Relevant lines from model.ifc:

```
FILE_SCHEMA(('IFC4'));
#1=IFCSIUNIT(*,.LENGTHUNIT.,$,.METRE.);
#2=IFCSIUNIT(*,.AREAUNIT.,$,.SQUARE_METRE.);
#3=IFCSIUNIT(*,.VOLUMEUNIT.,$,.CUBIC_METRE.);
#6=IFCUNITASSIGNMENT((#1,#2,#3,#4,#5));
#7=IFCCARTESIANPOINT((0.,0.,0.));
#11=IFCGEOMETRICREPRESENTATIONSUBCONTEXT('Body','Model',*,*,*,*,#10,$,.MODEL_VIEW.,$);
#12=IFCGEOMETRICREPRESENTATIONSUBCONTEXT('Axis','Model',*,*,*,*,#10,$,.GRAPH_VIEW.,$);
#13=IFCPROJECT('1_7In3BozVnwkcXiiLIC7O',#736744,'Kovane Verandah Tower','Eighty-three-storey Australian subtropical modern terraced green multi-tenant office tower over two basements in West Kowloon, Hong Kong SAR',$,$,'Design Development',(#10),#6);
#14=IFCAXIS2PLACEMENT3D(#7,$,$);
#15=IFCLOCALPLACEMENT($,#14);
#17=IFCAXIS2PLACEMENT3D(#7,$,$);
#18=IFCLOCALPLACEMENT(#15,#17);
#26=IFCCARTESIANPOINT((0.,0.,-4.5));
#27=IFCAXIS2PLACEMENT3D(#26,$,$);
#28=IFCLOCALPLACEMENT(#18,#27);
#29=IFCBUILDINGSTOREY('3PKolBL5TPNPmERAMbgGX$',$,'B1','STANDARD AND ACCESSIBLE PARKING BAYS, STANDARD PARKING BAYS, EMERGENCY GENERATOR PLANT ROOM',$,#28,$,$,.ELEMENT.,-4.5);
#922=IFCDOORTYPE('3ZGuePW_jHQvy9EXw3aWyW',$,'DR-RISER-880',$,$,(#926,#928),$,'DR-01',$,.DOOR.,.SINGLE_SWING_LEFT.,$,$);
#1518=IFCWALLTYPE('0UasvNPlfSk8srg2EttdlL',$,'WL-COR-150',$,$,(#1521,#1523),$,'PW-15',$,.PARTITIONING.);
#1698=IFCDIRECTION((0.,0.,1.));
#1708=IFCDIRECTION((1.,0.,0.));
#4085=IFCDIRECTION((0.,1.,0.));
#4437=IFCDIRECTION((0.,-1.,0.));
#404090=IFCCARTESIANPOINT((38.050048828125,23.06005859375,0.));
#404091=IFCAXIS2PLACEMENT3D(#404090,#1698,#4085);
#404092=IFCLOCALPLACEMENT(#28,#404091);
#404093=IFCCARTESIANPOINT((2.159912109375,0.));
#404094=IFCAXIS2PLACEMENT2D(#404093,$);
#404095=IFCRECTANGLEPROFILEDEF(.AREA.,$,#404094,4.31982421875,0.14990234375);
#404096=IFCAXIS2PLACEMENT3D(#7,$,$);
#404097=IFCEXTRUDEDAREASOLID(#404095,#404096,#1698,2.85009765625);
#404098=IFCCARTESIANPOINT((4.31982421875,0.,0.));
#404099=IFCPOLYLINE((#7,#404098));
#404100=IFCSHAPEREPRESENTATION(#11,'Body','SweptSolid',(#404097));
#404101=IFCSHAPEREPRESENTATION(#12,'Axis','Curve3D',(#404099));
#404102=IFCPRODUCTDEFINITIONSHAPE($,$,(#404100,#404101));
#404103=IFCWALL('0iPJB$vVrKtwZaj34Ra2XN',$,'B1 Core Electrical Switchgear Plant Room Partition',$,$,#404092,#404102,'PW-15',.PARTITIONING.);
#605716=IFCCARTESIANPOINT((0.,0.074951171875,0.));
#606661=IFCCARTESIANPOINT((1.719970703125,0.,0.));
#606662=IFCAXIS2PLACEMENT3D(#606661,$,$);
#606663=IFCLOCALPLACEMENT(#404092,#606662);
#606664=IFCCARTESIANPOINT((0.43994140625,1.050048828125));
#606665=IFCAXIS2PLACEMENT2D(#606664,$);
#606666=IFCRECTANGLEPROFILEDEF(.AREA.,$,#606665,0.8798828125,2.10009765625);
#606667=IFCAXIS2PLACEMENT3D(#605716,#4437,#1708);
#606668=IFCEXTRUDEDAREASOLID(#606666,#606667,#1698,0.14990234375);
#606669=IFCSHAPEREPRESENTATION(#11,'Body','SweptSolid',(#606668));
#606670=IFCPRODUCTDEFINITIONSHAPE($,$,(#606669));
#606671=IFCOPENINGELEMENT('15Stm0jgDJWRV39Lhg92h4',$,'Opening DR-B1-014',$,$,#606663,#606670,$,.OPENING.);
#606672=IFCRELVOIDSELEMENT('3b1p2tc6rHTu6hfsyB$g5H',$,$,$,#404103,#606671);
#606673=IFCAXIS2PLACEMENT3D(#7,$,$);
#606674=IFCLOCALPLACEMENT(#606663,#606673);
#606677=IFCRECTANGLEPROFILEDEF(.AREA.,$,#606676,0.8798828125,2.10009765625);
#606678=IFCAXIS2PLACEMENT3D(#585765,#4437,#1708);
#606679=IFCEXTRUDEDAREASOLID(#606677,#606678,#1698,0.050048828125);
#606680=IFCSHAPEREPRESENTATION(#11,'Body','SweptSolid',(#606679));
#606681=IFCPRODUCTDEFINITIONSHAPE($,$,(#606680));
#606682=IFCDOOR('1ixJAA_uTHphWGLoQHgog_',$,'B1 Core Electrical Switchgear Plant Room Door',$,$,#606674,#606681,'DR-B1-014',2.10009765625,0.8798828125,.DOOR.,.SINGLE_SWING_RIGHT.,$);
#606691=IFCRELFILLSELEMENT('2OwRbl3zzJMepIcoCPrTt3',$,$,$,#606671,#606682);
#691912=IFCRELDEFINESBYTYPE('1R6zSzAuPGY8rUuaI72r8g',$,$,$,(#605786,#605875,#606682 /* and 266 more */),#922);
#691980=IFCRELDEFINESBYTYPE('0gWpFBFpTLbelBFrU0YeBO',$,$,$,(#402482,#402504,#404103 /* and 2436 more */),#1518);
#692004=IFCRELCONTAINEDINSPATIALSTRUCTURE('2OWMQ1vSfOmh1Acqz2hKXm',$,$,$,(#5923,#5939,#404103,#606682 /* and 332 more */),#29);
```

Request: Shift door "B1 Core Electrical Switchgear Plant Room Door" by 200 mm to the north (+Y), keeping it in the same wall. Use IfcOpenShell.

```python
import ifcopenshell
import ifcopenshell.api.geometry
import ifcopenshell.util.placement
import ifcopenshell.util.unit

model = ifcopenshell.open("model.ifc")
unit_scale = ifcopenshell.util.unit.calculate_unit_scale(model)

door = model.by_guid("1ixJAA_uTHphWGLoQHgog_")
opening = door.FillsVoids[0].RelatingOpeningElement
wall = opening.VoidsElements[0].RelatingBuildingElement

wall_matrix = ifcopenshell.util.placement.get_local_placement(wall.ObjectPlacement)
shift = wall_matrix[:3, 0] * 0.2 / unit_scale
before = ifcopenshell.util.placement.get_local_placement(door.ObjectPlacement)[:3, 3].copy()

# The door is placed relative to its opening, so it follows when the opening moves.
matrix = ifcopenshell.util.placement.get_local_placement(opening.ObjectPlacement)
matrix[:3, 3] += shift
ifcopenshell.api.geometry.edit_object_placement(
    model, product=opening, matrix=matrix, is_si=False, should_transform_children=True
)

after = ifcopenshell.util.placement.get_local_placement(door.ObjectPlacement)[:3, 3]
print("door moved by", (after - before).round(3) + 0.0)

model.write("model-out.ifc")
```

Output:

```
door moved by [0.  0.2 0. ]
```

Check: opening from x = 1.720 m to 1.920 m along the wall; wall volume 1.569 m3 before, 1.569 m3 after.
